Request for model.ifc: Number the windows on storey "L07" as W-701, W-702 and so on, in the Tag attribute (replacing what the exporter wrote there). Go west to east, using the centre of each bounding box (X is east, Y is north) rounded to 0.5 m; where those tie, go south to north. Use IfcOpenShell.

First a look at what the model holds.

```python
import ifcopenshell
import ifcopenshell.util.element
import ifcopenshell.util.placement

model = ifcopenshell.open("model.ifc")
print(model.schema)
storey = next(s for s in model.by_type("IfcBuildingStorey") if s.Name == "L07")
windows = [e for e in ifcopenshell.util.element.get_decomposition(storey) if e.is_a("IfcWindow")]
for e in sorted(windows, key=lambda e: e.id()):
    origin = ifcopenshell.util.placement.get_local_placement(e.ObjectPlacement)[:3, 3]
    print(e.id(), e.Tag, e.Name, origin.round(2) + 0.0, sep=" | ")
```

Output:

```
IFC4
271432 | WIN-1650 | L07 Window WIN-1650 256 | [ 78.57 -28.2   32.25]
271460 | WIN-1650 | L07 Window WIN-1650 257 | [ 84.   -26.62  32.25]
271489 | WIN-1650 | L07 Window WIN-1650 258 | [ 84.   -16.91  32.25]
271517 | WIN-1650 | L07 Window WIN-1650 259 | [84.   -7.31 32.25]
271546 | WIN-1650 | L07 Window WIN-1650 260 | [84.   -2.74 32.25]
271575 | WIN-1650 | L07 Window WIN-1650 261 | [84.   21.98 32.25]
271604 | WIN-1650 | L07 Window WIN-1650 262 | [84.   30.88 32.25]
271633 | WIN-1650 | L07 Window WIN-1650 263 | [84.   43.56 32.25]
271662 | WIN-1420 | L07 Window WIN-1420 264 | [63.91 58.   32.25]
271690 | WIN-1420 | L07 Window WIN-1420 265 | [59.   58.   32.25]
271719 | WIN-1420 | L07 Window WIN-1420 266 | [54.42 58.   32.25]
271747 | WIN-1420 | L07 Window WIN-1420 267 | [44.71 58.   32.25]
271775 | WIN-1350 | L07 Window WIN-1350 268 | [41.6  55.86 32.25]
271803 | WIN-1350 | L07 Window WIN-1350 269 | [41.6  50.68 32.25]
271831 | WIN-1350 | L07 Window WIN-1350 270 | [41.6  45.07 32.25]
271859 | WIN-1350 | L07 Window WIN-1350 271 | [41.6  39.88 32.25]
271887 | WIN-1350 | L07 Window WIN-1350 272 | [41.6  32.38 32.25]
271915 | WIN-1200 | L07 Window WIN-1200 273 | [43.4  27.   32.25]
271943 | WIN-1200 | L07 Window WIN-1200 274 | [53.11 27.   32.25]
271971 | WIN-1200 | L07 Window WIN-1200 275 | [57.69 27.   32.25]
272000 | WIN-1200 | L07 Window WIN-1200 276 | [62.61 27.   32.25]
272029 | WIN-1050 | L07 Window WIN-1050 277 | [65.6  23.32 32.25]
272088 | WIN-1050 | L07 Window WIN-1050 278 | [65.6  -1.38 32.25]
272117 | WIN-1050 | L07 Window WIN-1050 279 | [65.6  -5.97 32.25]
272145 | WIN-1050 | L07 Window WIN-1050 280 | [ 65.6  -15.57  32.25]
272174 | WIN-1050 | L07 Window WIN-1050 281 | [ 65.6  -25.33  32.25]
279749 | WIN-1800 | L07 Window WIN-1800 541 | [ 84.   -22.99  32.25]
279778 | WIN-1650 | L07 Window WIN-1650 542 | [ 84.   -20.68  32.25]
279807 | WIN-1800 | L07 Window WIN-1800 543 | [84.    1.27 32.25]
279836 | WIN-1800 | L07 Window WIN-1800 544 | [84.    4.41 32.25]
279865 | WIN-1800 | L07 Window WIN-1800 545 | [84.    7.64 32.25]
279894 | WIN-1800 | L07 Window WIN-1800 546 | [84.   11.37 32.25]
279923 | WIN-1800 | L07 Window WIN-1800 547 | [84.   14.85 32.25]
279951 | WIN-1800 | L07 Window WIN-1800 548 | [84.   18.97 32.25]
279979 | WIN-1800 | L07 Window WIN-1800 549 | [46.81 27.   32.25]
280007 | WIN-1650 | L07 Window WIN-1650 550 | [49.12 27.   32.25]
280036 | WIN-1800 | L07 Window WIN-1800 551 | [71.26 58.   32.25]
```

```python
import ifcopenshell
import ifcopenshell.geom
import ifcopenshell.util.element
import ifcopenshell.util.shape

model = ifcopenshell.open("model.ifc")
settings = ifcopenshell.geom.settings()
settings.set("use-world-coords", True)


def centre(element):
    shape = ifcopenshell.geom.create_shape(settings, element)
    return ifcopenshell.util.shape.get_bbox_centroid(shape.geometry)


storey = next(s for s in model.by_type("IfcBuildingStorey") if s.Name == "L07")
windows = [e for e in ifcopenshell.util.element.get_decomposition(storey) if e.is_a("IfcWindow")]

# Insertion points can sit at a corner or the storey origin, so sort by the geometry (in metres).
centres = {e: centre(e) for e in windows}
windows.sort(key=lambda e: (round(centres[e][0] / 0.5), centres[e][1]))

for i, e in enumerate(windows, start=1):
    number = f"W-7{i:02d}"
    e.Tag = number
    print(e.id(), number)

model.write("model_updated.ifc")
```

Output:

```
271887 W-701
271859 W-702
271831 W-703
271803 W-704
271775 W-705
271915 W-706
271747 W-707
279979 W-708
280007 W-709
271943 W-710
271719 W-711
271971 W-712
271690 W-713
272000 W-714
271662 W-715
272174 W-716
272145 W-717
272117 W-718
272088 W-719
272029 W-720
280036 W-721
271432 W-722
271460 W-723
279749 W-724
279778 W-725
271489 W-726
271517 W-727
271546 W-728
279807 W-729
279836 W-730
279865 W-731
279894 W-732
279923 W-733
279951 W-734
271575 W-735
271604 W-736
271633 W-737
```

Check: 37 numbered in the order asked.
